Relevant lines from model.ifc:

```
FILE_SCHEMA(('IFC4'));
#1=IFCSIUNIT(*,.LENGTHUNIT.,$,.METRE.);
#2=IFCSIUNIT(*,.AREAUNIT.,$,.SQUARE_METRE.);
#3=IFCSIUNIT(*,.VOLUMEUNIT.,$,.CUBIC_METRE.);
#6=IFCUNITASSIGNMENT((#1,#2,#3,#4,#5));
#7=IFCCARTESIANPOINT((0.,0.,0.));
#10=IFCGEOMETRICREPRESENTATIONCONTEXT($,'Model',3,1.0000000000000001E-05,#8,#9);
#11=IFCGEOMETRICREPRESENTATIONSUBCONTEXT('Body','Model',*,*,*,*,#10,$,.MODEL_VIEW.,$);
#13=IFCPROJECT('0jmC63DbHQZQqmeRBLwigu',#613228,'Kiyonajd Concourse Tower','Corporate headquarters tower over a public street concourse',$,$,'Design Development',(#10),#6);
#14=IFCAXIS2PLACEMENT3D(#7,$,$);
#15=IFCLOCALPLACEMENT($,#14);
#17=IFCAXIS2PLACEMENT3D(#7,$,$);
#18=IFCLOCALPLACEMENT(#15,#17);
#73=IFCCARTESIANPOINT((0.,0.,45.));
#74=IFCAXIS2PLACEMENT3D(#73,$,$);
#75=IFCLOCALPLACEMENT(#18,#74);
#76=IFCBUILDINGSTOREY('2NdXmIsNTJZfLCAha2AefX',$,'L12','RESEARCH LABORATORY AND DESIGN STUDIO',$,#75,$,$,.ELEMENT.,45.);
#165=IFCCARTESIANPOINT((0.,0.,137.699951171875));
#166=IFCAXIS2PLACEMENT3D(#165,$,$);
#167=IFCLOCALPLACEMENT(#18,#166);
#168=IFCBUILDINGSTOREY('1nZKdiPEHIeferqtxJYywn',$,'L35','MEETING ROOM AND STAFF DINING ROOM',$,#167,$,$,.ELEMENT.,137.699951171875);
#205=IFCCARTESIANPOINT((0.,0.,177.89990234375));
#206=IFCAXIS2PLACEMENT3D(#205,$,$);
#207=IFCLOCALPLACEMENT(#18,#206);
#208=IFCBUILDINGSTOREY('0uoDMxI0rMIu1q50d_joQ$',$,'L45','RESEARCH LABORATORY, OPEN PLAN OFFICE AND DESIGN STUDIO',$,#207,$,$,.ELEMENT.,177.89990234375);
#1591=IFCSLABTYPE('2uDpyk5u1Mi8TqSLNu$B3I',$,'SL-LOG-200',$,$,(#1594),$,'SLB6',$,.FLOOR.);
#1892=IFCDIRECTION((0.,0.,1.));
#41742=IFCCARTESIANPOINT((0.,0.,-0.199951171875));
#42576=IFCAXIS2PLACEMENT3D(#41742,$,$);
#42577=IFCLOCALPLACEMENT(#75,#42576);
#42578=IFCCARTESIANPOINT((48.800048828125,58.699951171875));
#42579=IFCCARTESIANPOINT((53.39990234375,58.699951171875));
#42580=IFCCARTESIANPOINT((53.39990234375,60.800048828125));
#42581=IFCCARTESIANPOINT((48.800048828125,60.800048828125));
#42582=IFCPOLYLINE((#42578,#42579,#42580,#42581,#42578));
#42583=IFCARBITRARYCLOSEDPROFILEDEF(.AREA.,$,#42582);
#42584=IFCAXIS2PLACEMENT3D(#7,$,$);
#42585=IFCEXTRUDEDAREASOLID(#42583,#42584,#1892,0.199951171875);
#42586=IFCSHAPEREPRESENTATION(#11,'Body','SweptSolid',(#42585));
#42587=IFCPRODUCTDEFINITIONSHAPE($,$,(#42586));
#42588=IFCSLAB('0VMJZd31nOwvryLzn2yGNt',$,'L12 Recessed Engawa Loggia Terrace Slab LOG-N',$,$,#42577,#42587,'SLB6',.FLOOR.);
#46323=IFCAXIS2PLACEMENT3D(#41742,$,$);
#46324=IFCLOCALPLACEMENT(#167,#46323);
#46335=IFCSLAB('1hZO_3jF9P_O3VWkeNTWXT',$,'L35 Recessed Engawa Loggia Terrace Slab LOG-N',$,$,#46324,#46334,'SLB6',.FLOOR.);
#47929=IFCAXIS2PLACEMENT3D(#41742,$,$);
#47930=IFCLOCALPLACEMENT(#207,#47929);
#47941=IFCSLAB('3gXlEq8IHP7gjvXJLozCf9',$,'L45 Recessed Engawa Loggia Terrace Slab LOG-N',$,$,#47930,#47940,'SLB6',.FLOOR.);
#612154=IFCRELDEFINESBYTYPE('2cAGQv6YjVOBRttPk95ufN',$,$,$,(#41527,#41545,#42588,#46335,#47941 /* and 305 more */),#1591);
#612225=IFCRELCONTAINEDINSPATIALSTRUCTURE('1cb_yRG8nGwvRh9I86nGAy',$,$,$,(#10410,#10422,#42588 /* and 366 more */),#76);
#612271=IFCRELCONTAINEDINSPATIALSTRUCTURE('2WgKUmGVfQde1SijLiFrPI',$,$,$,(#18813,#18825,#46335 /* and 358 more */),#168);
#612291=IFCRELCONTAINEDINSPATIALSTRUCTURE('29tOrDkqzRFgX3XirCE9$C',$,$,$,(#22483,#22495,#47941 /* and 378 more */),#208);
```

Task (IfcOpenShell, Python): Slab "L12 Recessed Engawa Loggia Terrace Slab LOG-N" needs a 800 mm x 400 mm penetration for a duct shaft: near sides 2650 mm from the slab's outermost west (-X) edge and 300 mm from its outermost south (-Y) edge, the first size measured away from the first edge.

```python
import numpy as np
import ifcopenshell
import ifcopenshell.api.feature
import ifcopenshell.api.geometry
import ifcopenshell.api.root
import ifcopenshell.geom
import ifcopenshell.util.placement
import ifcopenshell.util.representation
import ifcopenshell.util.shape
import ifcopenshell.util.unit

model = ifcopenshell.open("model.ifc")
unit_scale = ifcopenshell.util.unit.calculate_unit_scale(model)
settings = ifcopenshell.geom.settings()


def volume(element):
    """Net volume in cubic metres, openings subtracted."""
    shape = ifcopenshell.geom.create_shape(settings, element)
    return ifcopenshell.util.shape.get_volume(shape.geometry)


slab = model.by_id(42588)
before = volume(slab)

# Extent in the slab's own axes, in metres. The edges named are its -X and -Y sides.
slab_shape = ifcopenshell.geom.create_shape(settings, slab)
vertices = ifcopenshell.util.shape.get_vertices(slab_shape.geometry)
x_min, y_min, bottom = vertices.min(axis=0)
top = vertices[:, 2].max()

opening = ifcopenshell.api.root.create_entity(model, ifc_class="IfcOpeningElement", name="Duct shaft opening", predefined_type="OPENING")
context = ifcopenshell.util.representation.get_context(model, "Model", "Body", "MODEL_VIEW")
width, depth = 0.8, 0.4
outline = [(0.0, 0.0), (width, 0.0), (width, depth), (0.0, depth), (0.0, 0.0)]
# Overshoot both faces by 50 mm so the cut is clean.
shape = ifcopenshell.api.geometry.add_slab_representation(
    model, context=context, depth=top - bottom + 0.1, polyline=outline
)
ifcopenshell.api.geometry.assign_representation(model, product=opening, representation=shape)

matrix = ifcopenshell.util.placement.get_local_placement(slab.ObjectPlacement)
matrix[:, 3] = matrix @ np.append(np.array([x_min + 2.65, y_min + 0.3, bottom - 0.05]) / unit_scale, 1.0)
ifcopenshell.api.geometry.edit_object_placement(model, product=opening, matrix=matrix, is_si=False)
ifcopenshell.api.feature.add_feature(model, feature=opening, element=slab)

after = volume(slab)

print(f"slab volume {before:.3f} -> {after:.3f} m3")

model.write("model_rev.ifc")
```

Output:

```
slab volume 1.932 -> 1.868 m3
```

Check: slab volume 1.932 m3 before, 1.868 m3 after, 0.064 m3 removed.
